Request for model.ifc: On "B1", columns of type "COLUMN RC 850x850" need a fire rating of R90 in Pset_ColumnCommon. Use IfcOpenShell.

First a look at what the model holds.

```python
import ifcopenshell
import ifcopenshell.util.element

model = ifcopenshell.open("model.ifc")
print(model.schema)
storey = next(s for s in model.by_type("IfcBuildingStorey") if s.Name == "B1")
columns = [e for e in ifcopenshell.util.element.get_decomposition(storey) if e.is_a("IfcColumn")]
seen = {}
for e in columns:
    element_type = ifcopenshell.util.element.get_type(e)
    key = (element_type.Name if element_type != e and element_type else None, ifcopenshell.util.element.get_pset(e, "Pset_ColumnCommon", "FireRating"))
    seen[key] = seen.get(key, 0) + 1
for (name, value), count in sorted(seen.items(), key=str):
    print(count, "x", name, "|", value)
```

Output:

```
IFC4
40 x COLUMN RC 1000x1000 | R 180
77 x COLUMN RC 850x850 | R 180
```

```python
import ifcopenshell
import ifcopenshell.api.pset
import ifcopenshell.util.element

model = ifcopenshell.open("model.ifc")

storey = next(s for s in model.by_type("IfcBuildingStorey") if s.Name == "B1")
columns = [e for e in ifcopenshell.util.element.get_decomposition(storey) if e.is_a("IfcColumn")]

count = 0
for e in columns:
    element_type = ifcopenshell.util.element.get_type(e)
    if element_type in (None, e) or element_type.Name != "COLUMN RC 850x850":
        continue
    # add_pset returns the element's existing set when there is one.
    pset = ifcopenshell.api.pset.add_pset(model, product=e, name="Pset_ColumnCommon")
    ifcopenshell.api.pset.edit_pset(model, pset=pset, properties={"FireRating": "R90"})
    count += 1

print(count, "columns updated")

model.write("model_updated.ifc")
```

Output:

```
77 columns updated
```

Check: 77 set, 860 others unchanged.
